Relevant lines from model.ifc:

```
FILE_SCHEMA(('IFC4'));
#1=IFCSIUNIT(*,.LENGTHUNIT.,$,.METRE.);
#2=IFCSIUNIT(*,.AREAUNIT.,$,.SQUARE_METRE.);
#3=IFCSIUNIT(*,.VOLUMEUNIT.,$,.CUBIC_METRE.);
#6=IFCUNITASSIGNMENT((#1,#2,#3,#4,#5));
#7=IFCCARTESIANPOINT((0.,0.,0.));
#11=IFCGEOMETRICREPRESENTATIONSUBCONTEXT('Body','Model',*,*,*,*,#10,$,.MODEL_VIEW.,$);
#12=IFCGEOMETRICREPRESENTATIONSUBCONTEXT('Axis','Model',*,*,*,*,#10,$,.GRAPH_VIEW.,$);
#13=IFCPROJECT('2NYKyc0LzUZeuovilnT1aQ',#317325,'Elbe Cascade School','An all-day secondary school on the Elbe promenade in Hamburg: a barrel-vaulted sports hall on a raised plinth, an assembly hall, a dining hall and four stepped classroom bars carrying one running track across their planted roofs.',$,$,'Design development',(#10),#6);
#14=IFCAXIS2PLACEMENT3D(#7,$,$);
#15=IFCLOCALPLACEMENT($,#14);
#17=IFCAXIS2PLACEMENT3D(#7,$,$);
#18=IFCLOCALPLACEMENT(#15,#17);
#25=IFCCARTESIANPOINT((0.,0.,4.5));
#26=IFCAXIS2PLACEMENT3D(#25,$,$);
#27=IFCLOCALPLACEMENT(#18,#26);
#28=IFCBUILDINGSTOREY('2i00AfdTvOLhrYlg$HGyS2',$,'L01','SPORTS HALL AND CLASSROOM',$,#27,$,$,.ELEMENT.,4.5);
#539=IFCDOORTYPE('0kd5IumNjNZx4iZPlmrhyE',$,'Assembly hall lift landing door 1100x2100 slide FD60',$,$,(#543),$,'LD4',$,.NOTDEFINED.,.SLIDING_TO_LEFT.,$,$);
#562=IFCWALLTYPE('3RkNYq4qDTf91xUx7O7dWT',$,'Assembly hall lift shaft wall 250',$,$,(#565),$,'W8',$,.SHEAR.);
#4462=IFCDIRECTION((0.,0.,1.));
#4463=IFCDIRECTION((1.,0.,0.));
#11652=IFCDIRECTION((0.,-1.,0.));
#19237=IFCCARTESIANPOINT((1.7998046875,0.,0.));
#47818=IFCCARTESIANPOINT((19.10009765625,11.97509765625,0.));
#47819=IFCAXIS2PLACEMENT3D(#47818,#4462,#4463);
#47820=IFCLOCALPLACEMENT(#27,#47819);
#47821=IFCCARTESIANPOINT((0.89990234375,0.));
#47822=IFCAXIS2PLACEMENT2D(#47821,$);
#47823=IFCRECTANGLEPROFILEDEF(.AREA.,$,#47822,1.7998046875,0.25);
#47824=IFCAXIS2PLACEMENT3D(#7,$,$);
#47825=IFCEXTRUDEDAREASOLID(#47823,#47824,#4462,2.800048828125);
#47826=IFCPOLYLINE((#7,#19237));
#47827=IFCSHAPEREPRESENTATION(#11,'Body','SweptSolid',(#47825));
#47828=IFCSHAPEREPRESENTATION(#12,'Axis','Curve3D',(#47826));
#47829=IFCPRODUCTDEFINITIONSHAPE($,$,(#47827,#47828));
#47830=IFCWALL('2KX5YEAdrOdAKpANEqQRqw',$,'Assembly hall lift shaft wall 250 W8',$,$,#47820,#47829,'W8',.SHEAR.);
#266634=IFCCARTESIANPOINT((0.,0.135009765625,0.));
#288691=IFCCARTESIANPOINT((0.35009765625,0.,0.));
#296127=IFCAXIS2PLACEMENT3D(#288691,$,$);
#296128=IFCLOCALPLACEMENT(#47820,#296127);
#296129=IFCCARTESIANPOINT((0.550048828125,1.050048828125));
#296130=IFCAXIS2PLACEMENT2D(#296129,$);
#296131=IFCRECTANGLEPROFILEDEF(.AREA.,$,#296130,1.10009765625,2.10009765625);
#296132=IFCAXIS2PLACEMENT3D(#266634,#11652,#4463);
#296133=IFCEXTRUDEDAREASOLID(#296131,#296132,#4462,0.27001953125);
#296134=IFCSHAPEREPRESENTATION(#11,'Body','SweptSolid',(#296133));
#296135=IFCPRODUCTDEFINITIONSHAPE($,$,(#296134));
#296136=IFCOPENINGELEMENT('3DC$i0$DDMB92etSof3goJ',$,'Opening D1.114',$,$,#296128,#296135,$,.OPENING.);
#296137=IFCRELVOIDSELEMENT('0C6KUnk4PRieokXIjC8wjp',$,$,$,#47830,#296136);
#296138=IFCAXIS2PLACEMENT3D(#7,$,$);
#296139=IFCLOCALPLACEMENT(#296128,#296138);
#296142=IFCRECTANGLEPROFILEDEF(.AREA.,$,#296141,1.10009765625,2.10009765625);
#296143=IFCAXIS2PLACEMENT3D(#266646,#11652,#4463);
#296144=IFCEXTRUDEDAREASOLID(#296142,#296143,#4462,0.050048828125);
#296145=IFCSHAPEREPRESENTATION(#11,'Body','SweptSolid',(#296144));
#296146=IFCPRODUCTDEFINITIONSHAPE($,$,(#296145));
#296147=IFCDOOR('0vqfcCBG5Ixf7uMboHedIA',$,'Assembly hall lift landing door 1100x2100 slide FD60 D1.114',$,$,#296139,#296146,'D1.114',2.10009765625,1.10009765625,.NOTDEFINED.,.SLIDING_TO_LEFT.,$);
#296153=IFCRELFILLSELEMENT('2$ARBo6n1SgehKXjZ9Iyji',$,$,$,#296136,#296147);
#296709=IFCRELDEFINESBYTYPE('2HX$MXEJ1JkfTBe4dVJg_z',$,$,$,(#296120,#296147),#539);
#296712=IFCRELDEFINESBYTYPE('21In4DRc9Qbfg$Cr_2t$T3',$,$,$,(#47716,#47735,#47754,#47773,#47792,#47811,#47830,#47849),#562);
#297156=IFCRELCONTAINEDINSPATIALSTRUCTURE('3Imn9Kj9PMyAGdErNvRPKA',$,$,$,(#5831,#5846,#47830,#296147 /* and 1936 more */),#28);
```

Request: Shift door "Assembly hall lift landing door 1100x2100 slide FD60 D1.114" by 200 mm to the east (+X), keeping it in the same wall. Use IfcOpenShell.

```python
import ifcopenshell
import ifcopenshell.api.geometry
import ifcopenshell.util.placement

model = ifcopenshell.open("model.ifc")

door = model.by_guid("0vqfcCBG5Ixf7uMboHedIA")
opening = door.FillsVoids[0].RelatingOpeningElement
wall = opening.VoidsElements[0].RelatingBuildingElement

wall_matrix = ifcopenshell.util.placement.get_local_placement(wall.ObjectPlacement)
shift = wall_matrix[:3, 0] * 0.2
before = ifcopenshell.util.placement.get_local_placement(door.ObjectPlacement)[:3, 3].copy()

# The door is placed relative to its opening, so it follows when the opening moves.
matrix = ifcopenshell.util.placement.get_local_placement(opening.ObjectPlacement)
matrix[:3, 3] += shift
ifcopenshell.api.geometry.edit_object_placement(
    model, product=opening, matrix=matrix, is_si=False, should_transform_children=True
)

after = ifcopenshell.util.placement.get_local_placement(door.ObjectPlacement)[:3, 3]
print("door moved by", (after - before).round(3) + 0.0)

model.write("model_edited.ifc")
```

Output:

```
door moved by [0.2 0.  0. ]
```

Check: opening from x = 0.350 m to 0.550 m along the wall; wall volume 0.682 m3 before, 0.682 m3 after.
